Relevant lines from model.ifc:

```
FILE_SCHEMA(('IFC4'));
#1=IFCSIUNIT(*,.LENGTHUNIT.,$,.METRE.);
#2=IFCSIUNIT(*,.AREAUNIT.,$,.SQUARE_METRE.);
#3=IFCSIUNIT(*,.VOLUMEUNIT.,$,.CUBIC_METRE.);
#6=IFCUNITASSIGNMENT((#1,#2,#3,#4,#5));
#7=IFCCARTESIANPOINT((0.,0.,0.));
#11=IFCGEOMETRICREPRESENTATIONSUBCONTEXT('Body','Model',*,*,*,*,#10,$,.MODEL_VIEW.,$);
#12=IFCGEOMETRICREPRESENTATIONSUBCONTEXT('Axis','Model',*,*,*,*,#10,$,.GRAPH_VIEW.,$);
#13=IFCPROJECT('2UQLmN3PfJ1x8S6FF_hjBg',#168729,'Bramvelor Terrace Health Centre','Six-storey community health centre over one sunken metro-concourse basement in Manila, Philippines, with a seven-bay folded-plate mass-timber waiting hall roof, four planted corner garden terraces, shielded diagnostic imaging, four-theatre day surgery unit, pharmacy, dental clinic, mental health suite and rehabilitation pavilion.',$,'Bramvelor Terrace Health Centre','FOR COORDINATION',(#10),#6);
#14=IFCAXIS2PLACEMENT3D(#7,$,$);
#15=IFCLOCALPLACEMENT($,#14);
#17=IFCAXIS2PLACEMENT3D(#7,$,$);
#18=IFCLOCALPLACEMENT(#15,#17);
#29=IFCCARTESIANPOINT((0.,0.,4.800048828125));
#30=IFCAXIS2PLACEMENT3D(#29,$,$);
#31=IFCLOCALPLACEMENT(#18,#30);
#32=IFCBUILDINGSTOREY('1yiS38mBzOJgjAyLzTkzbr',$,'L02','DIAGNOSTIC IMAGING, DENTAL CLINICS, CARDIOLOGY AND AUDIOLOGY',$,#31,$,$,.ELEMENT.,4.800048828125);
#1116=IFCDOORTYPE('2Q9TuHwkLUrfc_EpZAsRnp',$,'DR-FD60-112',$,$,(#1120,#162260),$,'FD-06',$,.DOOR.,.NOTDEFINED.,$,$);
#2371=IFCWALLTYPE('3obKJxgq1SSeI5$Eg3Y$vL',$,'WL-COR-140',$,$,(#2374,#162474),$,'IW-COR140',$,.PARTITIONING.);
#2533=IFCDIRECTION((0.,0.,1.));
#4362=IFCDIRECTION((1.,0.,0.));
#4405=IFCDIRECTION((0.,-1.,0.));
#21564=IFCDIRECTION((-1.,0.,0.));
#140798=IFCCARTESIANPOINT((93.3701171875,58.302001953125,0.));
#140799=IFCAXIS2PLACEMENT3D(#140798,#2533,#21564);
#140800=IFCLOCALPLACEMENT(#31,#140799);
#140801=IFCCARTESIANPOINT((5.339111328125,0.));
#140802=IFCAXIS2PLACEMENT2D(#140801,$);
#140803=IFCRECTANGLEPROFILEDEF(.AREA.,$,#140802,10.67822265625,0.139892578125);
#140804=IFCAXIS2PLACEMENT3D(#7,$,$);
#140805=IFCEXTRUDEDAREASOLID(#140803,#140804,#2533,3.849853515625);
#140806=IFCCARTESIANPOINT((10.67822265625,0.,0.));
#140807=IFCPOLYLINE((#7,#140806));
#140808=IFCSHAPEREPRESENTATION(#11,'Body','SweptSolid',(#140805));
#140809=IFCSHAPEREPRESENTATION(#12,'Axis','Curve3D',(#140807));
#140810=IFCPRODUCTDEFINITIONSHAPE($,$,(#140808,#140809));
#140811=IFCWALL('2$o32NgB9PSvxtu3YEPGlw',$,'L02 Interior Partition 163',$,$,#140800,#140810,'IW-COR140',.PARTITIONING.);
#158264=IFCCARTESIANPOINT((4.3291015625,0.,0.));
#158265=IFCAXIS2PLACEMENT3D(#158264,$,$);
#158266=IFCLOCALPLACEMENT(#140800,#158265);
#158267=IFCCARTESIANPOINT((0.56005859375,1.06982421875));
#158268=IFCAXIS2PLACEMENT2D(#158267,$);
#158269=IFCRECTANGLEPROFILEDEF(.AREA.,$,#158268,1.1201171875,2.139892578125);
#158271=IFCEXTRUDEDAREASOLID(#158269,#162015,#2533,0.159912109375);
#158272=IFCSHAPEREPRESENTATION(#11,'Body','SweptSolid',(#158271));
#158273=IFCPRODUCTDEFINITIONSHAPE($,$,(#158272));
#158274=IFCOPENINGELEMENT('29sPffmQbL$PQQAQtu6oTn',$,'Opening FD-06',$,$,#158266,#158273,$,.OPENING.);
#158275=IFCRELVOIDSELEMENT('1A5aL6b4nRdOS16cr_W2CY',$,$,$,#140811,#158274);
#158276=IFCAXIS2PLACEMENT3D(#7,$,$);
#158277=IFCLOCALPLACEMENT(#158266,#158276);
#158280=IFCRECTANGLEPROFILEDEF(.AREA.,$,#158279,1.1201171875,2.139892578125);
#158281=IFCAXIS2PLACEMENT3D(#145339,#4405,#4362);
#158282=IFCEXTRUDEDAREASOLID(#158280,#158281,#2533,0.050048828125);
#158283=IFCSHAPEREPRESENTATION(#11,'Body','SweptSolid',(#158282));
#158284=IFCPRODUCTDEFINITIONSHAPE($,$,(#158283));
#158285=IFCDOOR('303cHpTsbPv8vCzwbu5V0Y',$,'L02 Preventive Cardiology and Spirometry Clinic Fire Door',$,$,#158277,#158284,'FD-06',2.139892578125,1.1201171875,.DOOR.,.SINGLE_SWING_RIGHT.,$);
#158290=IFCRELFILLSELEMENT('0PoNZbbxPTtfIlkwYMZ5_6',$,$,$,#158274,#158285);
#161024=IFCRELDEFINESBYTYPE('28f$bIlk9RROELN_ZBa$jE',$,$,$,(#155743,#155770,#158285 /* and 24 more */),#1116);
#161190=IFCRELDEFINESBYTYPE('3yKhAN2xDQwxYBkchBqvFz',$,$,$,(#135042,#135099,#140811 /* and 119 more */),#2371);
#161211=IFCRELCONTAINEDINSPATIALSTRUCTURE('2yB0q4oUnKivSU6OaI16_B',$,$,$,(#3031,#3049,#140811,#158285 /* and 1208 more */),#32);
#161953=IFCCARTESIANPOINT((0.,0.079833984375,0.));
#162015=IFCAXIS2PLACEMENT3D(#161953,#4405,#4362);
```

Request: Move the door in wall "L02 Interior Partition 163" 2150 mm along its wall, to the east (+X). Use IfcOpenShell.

```python
import ifcopenshell
import ifcopenshell.api.geometry
import ifcopenshell.util.placement
import ifcopenshell.util.unit

model = ifcopenshell.open("model.ifc")
unit_scale = ifcopenshell.util.unit.calculate_unit_scale(model)

door = model.by_id(158285)
opening = door.FillsVoids[0].RelatingOpeningElement
wall = opening.VoidsElements[0].RelatingBuildingElement

wall_matrix = ifcopenshell.util.placement.get_local_placement(wall.ObjectPlacement)
shift = wall_matrix[:3, 0] * -2.15 / unit_scale
before = ifcopenshell.util.placement.get_local_placement(door.ObjectPlacement)[:3, 3].copy()

# The door is placed relative to its opening, so it follows when the opening moves.
matrix = ifcopenshell.util.placement.get_local_placement(opening.ObjectPlacement)
matrix[:3, 3] += shift
ifcopenshell.api.geometry.edit_object_placement(
    model, product=opening, matrix=matrix, is_si=False, should_transform_children=True
)

after = ifcopenshell.util.placement.get_local_placement(door.ObjectPlacement)[:3, 3]
print("door moved by", (after - before).round(3) + 0.0)

model.write("model_rev.ifc")
```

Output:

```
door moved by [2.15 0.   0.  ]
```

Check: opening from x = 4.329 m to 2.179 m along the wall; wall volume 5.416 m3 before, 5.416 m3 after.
